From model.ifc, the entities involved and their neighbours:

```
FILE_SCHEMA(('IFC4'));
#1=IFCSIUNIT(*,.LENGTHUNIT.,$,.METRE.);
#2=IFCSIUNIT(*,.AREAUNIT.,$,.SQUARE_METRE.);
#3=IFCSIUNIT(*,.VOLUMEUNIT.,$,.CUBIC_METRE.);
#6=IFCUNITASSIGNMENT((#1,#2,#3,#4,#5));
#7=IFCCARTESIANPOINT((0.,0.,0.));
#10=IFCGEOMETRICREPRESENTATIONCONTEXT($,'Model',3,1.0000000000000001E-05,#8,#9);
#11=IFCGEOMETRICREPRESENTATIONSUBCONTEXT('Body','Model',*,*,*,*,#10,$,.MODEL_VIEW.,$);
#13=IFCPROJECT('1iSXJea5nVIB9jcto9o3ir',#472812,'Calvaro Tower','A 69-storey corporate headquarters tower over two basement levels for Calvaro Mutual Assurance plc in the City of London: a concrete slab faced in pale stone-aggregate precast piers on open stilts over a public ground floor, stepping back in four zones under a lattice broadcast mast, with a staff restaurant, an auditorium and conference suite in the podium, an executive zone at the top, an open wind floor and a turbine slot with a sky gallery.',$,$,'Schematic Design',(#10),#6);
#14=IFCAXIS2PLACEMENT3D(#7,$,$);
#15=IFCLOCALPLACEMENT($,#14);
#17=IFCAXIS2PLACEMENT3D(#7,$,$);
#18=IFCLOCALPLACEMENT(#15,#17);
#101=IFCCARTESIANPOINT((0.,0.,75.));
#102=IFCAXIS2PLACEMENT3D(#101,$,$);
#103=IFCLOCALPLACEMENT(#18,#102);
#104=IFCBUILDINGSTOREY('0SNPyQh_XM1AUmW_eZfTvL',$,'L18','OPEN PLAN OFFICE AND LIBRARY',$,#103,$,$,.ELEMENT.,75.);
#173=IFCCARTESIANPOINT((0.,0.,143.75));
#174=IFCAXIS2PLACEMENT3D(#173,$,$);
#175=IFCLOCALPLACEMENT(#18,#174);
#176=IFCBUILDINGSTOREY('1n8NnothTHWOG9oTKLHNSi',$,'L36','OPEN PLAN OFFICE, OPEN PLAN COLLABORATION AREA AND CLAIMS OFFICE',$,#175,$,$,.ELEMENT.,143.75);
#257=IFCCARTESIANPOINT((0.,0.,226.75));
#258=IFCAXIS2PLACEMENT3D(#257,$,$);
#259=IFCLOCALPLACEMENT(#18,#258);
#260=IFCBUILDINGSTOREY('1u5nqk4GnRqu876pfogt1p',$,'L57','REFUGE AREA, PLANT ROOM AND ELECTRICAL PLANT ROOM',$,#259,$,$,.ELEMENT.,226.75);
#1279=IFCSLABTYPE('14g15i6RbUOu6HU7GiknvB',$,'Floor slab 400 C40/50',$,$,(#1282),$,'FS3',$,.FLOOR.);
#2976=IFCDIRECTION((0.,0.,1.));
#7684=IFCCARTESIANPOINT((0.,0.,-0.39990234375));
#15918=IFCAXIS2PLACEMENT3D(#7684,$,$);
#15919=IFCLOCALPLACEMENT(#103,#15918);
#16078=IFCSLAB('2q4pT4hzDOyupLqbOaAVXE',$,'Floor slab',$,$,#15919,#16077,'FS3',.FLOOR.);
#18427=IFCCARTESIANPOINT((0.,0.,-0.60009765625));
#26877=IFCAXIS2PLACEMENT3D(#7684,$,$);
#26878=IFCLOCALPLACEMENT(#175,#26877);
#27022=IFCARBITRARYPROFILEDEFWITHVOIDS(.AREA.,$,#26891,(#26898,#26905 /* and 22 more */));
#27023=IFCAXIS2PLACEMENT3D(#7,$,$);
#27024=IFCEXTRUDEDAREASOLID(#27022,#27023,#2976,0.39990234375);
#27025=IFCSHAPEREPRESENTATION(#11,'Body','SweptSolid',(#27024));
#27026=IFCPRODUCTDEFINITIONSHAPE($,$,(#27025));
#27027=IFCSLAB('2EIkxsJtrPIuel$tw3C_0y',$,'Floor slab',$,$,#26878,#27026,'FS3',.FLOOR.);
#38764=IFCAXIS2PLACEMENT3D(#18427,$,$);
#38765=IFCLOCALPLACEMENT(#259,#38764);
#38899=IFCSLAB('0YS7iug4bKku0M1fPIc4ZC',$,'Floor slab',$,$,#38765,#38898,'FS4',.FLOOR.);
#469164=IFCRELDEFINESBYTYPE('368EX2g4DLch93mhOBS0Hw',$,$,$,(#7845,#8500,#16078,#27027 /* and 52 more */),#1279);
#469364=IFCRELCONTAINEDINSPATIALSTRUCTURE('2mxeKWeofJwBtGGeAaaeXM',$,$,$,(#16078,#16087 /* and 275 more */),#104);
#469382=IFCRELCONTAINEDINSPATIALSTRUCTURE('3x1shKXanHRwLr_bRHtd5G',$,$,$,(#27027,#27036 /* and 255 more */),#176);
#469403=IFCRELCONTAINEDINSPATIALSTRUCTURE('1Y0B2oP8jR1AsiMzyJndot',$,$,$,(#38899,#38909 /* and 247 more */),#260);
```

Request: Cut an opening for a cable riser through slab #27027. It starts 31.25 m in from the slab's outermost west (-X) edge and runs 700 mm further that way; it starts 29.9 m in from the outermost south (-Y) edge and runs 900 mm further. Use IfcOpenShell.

```python
import numpy as np
import ifcopenshell
import ifcopenshell.api.feature
import ifcopenshell.api.geometry
import ifcopenshell.api.root
import ifcopenshell.geom
import ifcopenshell.util.placement
import ifcopenshell.util.representation
import ifcopenshell.util.shape
import ifcopenshell.util.unit

model = ifcopenshell.open("model.ifc")
unit_scale = ifcopenshell.util.unit.calculate_unit_scale(model)
settings = ifcopenshell.geom.settings()


def volume(element):
    """Net volume in cubic metres, openings subtracted."""
    shape = ifcopenshell.geom.create_shape(settings, element)
    return ifcopenshell.util.shape.get_volume(shape.geometry)


slab = model.by_id(27027)
before = volume(slab)

# Extent in the slab's own axes, in metres. The edges named are its -X and -Y sides.
slab_shape = ifcopenshell.geom.create_shape(settings, slab)
vertices = ifcopenshell.util.shape.get_vertices(slab_shape.geometry)
x_min, y_min, bottom = vertices.min(axis=0)
top = vertices[:, 2].max()

opening = ifcopenshell.api.root.create_entity(model, ifc_class="IfcOpeningElement", name="Cable riser opening", predefined_type="OPENING")
context = ifcopenshell.util.representation.get_context(model, "Model", "Body", "MODEL_VIEW")
width, depth = 0.7, 0.9
outline = [(0.0, 0.0), (width, 0.0), (width, depth), (0.0, depth), (0.0, 0.0)]
# Overshoot both faces by 50 mm so the cut is clean.
shape = ifcopenshell.api.geometry.add_slab_representation(
    model, context=context, depth=top - bottom + 0.1, polyline=outline
)
ifcopenshell.api.geometry.assign_representation(model, product=opening, representation=shape)

matrix = ifcopenshell.util.placement.get_local_placement(slab.ObjectPlacement)
matrix[:, 3] = matrix @ np.append(np.array([x_min + 31.25, y_min + 29.9, bottom - 0.05]) / unit_scale, 1.0)
ifcopenshell.api.geometry.edit_object_placement(model, product=opening, matrix=matrix, is_si=False)
ifcopenshell.api.feature.add_feature(model, feature=opening, element=slab)

after = volume(slab)

print(f"slab volume {before:.3f} -> {after:.3f} m3")

model.write("model_rev.ifc")
```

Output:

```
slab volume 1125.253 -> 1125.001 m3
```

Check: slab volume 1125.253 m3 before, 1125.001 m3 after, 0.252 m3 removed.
